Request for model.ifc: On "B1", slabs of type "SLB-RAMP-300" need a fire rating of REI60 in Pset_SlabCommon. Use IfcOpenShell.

First a look at what the model holds.

```python
import ifcopenshell
import ifcopenshell.util.element

model = ifcopenshell.open("model.ifc")
print(model.schema)
storey = next(s for s in model.by_type("IfcBuildingStorey") if s.Name == "B1")
slabs = [e for e in ifcopenshell.util.element.get_decomposition(storey) if e.is_a("IfcSlab")]
seen = {}
for e in slabs:
    element_type = ifcopenshell.util.element.get_type(e)
    key = (element_type.Name if element_type != e and element_type else None, ifcopenshell.util.element.get_pset(e, "Pset_SlabCommon", "FireRating"))
    seen[key] = seen.get(key, 0) + 1
for (name, value), count in sorted(seen.items(), key=str):
    print(count, "x", name, "|", value)
```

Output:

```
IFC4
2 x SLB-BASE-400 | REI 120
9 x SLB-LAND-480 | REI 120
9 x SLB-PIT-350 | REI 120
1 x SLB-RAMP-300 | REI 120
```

```python
import ifcopenshell
import ifcopenshell.api.pset
import ifcopenshell.util.element

model = ifcopenshell.open("model.ifc")

storey = next(s for s in model.by_type("IfcBuildingStorey") if s.Name == "B1")
slabs = [e for e in ifcopenshell.util.element.get_decomposition(storey) if e.is_a("IfcSlab")]

count = 0
for e in slabs:
    element_type = ifcopenshell.util.element.get_type(e)
    if element_type in (None, e) or element_type.Name != "SLB-RAMP-300":
        continue
    # add_pset returns the element's existing set when there is one.
    pset = ifcopenshell.api.pset.add_pset(model, product=e, name="Pset_SlabCommon")
    ifcopenshell.api.pset.edit_pset(model, pset=pset, properties={"FireRating": "REI60"})
    count += 1

print(count, "slabs updated")

model.write("model_rev.ifc")
```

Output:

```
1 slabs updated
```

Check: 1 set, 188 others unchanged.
